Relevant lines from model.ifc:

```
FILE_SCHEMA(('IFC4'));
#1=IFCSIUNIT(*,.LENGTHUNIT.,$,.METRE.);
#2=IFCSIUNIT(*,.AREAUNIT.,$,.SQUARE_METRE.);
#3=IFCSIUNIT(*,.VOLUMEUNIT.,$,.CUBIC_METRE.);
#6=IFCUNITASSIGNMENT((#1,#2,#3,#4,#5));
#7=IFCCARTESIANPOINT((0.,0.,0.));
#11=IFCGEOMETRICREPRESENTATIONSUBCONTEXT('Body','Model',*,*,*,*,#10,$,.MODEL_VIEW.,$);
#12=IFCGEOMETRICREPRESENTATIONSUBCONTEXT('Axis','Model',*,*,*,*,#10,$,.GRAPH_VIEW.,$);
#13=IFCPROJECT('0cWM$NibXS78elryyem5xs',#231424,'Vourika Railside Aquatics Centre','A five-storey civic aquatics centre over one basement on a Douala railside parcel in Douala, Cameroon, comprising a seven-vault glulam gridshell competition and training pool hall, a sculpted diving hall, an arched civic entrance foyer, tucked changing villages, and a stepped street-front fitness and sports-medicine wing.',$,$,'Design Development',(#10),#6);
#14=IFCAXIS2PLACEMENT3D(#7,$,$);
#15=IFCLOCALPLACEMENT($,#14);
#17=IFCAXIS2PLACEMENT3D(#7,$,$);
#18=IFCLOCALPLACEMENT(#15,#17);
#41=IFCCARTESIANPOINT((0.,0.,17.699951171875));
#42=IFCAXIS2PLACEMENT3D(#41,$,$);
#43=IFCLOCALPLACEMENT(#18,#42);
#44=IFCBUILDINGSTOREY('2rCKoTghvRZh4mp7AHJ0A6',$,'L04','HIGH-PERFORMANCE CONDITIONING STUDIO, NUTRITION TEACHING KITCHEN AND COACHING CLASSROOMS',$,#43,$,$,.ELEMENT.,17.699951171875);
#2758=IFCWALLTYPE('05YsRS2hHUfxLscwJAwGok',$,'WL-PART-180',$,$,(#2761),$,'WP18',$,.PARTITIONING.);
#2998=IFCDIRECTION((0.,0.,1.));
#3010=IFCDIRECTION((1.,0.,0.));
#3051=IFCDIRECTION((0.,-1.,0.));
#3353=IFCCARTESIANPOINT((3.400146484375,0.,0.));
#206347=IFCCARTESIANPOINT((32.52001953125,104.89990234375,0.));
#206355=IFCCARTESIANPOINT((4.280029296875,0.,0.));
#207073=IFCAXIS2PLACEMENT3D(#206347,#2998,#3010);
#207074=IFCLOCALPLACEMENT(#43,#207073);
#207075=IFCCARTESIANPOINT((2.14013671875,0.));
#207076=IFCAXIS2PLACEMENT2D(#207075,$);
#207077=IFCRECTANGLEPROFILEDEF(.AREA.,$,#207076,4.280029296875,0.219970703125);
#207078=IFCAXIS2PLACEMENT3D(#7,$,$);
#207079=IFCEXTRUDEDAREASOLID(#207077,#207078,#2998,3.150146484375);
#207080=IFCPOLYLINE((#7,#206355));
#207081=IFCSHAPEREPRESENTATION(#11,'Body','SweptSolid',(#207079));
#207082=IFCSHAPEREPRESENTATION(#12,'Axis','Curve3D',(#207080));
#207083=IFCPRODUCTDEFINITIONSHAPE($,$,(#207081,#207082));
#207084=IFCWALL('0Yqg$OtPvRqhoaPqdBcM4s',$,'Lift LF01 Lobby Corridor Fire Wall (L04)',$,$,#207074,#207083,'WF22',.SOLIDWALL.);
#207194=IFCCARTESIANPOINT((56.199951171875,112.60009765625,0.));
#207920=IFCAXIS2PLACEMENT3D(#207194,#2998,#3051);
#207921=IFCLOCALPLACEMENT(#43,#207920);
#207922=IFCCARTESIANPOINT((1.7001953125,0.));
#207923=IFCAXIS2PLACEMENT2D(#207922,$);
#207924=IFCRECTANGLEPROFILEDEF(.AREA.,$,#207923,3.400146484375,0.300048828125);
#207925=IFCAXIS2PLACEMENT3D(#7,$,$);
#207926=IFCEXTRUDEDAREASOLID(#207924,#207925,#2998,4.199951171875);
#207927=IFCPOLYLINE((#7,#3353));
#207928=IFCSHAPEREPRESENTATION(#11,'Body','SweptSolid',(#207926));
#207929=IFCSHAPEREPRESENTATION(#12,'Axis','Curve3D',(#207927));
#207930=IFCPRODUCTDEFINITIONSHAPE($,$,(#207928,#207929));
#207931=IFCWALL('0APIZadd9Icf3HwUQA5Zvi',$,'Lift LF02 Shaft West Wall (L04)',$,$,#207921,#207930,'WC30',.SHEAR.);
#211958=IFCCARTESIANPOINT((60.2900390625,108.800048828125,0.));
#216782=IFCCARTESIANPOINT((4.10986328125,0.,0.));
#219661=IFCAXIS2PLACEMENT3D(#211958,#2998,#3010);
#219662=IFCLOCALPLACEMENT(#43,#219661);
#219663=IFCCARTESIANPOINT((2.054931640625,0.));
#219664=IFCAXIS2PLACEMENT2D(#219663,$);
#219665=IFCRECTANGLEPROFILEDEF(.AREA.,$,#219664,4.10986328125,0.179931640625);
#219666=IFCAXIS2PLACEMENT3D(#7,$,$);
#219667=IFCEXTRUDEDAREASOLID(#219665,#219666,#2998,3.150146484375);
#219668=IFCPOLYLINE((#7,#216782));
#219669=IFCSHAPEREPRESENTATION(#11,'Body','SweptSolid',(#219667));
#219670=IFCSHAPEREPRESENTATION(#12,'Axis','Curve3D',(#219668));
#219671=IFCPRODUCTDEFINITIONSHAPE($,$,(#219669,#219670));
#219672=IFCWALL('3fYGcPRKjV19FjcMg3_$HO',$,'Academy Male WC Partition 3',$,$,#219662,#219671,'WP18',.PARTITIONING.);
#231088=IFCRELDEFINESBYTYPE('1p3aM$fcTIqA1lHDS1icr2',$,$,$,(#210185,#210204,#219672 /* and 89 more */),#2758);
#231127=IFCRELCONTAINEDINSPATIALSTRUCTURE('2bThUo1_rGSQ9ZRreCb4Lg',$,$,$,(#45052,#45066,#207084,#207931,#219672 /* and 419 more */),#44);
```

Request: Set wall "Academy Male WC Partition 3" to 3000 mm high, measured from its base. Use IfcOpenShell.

```python
import ifcopenshell
import ifcopenshell.geom
import ifcopenshell.util.representation
import ifcopenshell.util.shape

model = ifcopenshell.open("model.ifc")
settings = ifcopenshell.geom.settings()


def volume(element):
    """Net volume in cubic metres, openings subtracted."""
    shape = ifcopenshell.geom.create_shape(settings, element)
    return ifcopenshell.util.shape.get_volume(shape.geometry)


wall = model.by_guid("3fYGcPRKjV19FjcMg3_$HO")
before = volume(wall)

body = ifcopenshell.util.representation.get_representation(wall, "Model", "Body")
solid = body.Items[0]
old_height = solid.Depth
solid.Depth = 3.0
after = volume(wall)

print(f"height {old_height:g} -> {solid.Depth:g}, volume {before:.3f} -> {after:.3f} m3")

model.write("model_updated.ifc")
```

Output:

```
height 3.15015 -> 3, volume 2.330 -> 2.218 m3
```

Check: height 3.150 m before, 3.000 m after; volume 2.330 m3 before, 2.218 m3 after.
